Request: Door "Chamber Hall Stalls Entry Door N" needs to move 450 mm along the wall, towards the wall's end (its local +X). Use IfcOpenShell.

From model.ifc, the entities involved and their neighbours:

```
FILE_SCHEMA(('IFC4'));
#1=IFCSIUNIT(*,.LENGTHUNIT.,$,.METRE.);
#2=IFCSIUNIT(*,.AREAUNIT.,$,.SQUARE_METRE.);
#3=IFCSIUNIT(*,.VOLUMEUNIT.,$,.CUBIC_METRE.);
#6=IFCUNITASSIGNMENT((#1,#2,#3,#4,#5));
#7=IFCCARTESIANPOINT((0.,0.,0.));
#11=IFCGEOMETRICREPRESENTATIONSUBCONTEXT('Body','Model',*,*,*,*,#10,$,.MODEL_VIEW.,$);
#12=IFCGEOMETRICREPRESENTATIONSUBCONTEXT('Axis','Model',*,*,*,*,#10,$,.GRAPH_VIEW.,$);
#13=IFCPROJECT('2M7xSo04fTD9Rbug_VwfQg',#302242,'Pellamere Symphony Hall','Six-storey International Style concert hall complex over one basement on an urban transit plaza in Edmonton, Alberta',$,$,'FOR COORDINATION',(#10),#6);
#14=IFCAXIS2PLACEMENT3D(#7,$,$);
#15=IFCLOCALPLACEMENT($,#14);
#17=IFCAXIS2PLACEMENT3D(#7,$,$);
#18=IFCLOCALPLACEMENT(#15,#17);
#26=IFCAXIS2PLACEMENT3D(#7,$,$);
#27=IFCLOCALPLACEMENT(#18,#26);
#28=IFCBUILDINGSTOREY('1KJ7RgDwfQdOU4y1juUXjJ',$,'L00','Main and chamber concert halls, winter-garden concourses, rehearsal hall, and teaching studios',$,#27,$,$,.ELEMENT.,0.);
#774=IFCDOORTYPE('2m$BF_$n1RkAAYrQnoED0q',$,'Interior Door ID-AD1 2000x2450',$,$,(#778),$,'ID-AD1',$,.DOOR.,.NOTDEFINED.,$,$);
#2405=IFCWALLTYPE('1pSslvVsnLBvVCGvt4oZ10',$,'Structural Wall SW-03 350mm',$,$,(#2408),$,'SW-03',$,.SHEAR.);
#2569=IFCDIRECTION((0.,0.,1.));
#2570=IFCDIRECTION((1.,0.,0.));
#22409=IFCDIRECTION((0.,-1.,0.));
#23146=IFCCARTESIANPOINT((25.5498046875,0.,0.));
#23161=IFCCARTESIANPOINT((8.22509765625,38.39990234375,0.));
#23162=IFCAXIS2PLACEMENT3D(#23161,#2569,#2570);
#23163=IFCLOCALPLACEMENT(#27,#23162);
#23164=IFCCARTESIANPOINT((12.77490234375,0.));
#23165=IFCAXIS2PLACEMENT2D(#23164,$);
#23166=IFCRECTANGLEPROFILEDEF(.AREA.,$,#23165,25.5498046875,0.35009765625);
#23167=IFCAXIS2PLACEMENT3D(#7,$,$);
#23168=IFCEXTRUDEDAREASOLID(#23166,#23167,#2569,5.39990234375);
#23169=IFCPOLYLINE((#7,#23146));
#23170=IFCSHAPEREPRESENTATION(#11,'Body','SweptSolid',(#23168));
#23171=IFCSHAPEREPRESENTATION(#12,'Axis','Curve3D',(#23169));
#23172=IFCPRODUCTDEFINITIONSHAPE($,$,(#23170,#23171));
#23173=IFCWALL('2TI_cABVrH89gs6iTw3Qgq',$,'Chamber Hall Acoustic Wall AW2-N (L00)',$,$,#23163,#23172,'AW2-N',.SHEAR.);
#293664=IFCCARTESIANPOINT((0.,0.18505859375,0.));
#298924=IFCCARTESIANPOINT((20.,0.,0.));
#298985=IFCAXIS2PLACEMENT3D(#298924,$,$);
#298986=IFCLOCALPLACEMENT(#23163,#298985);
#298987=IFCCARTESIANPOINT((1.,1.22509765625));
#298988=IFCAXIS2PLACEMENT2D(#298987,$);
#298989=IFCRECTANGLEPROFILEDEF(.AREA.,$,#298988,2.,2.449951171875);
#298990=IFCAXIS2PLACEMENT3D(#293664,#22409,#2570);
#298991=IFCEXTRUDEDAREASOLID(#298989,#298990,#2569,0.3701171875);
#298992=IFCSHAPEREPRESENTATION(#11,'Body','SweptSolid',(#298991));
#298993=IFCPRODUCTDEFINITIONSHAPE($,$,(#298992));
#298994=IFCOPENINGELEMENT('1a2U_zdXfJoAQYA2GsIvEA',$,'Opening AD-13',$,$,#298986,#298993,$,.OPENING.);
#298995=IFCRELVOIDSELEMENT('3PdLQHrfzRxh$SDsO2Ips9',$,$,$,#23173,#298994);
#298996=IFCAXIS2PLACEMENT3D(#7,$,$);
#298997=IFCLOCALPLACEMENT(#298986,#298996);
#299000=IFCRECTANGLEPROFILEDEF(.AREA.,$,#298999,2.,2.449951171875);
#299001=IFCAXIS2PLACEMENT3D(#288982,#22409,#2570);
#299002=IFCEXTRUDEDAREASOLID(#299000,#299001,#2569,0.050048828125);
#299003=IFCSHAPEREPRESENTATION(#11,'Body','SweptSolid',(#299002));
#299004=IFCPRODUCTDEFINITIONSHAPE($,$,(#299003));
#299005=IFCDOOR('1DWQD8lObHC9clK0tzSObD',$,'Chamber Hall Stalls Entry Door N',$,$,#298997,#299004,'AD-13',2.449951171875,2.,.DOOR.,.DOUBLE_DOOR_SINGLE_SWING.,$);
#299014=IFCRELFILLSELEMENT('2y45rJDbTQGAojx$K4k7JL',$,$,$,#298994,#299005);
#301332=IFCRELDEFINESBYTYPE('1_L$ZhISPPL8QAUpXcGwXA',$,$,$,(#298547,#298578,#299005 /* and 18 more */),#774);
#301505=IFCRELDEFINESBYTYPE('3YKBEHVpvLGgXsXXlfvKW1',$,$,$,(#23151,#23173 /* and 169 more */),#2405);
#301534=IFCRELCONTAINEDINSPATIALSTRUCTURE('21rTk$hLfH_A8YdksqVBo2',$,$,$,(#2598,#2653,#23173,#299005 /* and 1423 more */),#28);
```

```python
import ifcopenshell
import ifcopenshell.api.geometry
import ifcopenshell.util.placement

model = ifcopenshell.open("model.ifc")

door = model.by_guid("1DWQD8lObHC9clK0tzSObD")
opening = door.FillsVoids[0].RelatingOpeningElement
wall = opening.VoidsElements[0].RelatingBuildingElement

wall_matrix = ifcopenshell.util.placement.get_local_placement(wall.ObjectPlacement)
shift = wall_matrix[:3, 0] * 0.45
before = ifcopenshell.util.placement.get_local_placement(door.ObjectPlacement)[:3, 3].copy()

# The door is placed relative to its opening, so it follows when the opening moves.
matrix = ifcopenshell.util.placement.get_local_placement(opening.ObjectPlacement)
matrix[:3, 3] += shift
ifcopenshell.api.geometry.edit_object_placement(
    model, product=opening, matrix=matrix, is_si=False, should_transform_children=True
)

after = ifcopenshell.util.placement.get_local_placement(door.ObjectPlacement)[:3, 3]
print("door moved by", (after - before).round(3) + 0.0)

model.write("model_updated.ifc")
```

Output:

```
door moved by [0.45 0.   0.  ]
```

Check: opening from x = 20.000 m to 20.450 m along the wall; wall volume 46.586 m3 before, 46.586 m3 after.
